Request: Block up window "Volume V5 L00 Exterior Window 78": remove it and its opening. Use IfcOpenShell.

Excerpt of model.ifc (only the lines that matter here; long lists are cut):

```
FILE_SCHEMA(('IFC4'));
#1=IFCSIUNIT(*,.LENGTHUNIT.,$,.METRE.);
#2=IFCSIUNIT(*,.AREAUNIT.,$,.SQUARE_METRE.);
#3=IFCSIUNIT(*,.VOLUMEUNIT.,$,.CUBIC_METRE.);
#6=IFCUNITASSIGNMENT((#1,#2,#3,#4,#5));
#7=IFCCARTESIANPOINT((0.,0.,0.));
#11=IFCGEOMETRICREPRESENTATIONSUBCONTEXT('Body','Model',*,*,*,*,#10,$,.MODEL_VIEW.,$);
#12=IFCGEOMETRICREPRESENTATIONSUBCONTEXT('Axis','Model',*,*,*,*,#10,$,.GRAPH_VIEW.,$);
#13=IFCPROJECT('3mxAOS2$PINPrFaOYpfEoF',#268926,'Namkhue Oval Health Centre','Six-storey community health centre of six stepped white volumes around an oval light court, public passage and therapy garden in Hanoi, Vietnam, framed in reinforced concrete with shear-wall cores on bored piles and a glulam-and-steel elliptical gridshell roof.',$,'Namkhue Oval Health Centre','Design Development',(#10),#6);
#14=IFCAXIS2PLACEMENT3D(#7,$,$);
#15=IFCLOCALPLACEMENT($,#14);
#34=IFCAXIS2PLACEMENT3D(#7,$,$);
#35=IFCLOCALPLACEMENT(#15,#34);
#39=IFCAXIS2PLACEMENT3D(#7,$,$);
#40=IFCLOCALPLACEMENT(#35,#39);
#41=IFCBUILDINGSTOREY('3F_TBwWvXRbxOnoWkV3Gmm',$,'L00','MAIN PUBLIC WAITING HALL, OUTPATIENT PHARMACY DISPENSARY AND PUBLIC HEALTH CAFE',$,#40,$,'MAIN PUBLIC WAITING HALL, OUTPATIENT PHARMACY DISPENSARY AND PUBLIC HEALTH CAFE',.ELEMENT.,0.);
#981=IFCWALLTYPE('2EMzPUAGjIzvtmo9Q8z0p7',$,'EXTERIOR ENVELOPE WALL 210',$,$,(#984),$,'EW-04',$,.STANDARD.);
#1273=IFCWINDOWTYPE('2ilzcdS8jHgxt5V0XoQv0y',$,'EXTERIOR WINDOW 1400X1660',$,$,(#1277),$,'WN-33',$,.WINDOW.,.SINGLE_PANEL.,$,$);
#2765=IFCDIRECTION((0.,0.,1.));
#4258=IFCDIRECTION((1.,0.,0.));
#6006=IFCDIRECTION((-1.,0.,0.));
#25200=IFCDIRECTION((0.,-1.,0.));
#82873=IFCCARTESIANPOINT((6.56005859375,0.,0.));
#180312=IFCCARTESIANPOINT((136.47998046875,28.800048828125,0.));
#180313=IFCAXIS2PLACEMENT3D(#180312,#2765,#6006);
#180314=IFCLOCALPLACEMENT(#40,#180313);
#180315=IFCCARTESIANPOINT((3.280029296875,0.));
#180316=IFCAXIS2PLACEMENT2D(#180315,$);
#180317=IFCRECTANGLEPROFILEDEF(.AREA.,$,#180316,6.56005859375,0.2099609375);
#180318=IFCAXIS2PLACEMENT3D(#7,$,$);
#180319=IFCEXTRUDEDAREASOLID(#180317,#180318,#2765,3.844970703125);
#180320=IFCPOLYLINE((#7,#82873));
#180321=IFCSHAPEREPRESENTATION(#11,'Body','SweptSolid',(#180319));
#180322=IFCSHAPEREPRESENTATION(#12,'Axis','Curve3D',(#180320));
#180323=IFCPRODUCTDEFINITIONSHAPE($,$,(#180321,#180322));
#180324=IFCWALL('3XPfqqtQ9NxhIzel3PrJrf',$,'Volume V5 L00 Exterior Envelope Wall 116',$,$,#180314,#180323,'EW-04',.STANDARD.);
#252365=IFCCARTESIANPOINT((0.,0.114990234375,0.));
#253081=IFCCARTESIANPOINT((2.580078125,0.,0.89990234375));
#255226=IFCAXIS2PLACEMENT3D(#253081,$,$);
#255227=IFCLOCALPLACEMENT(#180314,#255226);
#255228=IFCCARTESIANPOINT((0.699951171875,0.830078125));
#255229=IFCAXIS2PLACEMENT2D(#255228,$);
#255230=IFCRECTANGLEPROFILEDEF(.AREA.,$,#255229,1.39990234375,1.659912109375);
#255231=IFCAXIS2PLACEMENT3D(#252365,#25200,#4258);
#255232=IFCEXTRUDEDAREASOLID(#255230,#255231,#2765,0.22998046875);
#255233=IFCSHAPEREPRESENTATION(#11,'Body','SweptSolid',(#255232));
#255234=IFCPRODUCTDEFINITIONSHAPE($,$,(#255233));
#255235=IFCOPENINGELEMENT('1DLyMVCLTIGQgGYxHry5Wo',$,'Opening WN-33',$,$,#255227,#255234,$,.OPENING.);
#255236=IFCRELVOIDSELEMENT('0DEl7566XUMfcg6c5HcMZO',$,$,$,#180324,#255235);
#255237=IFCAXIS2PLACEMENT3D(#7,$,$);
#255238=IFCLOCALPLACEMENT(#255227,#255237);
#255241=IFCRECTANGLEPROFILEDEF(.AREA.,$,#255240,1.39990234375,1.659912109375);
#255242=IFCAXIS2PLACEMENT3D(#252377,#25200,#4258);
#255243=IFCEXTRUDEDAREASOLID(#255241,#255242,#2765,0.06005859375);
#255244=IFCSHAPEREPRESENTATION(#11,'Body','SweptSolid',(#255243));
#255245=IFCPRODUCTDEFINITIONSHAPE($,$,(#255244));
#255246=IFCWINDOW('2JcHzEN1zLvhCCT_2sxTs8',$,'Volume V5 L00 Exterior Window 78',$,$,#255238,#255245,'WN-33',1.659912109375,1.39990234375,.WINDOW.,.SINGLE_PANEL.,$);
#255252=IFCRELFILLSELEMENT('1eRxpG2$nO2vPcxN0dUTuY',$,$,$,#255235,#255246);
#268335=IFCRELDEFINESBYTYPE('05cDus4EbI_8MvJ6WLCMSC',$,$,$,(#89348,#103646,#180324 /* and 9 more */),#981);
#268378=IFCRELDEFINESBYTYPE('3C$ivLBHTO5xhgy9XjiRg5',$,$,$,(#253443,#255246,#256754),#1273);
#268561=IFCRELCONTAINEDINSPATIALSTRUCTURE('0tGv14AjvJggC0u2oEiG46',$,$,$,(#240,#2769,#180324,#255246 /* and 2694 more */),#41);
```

```python
import ifcopenshell
import ifcopenshell.api.feature
import ifcopenshell.api.root
import ifcopenshell.geom
import ifcopenshell.util.shape

model = ifcopenshell.open("model.ifc")
settings = ifcopenshell.geom.settings()


def volume(element):
    """Net volume in cubic metres, openings subtracted."""
    shape = ifcopenshell.geom.create_shape(settings, element)
    return ifcopenshell.util.shape.get_volume(shape.geometry)


window = model.by_guid("2JcHzEN1zLvhCCT_2sxTs8")
opening = window.FillsVoids[0].RelatingOpeningElement
wall = opening.VoidsElements[0].RelatingBuildingElement
before = volume(wall)

ifcopenshell.api.root.remove_product(model, product=window)
ifcopenshell.api.feature.remove_feature(model, feature=opening)

after = volume(wall)

print(f"wall volume {before:.3f} -> {after:.3f} m3")

model.write("model_updated.ifc")
```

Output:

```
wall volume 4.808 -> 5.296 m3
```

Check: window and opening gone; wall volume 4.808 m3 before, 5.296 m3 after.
